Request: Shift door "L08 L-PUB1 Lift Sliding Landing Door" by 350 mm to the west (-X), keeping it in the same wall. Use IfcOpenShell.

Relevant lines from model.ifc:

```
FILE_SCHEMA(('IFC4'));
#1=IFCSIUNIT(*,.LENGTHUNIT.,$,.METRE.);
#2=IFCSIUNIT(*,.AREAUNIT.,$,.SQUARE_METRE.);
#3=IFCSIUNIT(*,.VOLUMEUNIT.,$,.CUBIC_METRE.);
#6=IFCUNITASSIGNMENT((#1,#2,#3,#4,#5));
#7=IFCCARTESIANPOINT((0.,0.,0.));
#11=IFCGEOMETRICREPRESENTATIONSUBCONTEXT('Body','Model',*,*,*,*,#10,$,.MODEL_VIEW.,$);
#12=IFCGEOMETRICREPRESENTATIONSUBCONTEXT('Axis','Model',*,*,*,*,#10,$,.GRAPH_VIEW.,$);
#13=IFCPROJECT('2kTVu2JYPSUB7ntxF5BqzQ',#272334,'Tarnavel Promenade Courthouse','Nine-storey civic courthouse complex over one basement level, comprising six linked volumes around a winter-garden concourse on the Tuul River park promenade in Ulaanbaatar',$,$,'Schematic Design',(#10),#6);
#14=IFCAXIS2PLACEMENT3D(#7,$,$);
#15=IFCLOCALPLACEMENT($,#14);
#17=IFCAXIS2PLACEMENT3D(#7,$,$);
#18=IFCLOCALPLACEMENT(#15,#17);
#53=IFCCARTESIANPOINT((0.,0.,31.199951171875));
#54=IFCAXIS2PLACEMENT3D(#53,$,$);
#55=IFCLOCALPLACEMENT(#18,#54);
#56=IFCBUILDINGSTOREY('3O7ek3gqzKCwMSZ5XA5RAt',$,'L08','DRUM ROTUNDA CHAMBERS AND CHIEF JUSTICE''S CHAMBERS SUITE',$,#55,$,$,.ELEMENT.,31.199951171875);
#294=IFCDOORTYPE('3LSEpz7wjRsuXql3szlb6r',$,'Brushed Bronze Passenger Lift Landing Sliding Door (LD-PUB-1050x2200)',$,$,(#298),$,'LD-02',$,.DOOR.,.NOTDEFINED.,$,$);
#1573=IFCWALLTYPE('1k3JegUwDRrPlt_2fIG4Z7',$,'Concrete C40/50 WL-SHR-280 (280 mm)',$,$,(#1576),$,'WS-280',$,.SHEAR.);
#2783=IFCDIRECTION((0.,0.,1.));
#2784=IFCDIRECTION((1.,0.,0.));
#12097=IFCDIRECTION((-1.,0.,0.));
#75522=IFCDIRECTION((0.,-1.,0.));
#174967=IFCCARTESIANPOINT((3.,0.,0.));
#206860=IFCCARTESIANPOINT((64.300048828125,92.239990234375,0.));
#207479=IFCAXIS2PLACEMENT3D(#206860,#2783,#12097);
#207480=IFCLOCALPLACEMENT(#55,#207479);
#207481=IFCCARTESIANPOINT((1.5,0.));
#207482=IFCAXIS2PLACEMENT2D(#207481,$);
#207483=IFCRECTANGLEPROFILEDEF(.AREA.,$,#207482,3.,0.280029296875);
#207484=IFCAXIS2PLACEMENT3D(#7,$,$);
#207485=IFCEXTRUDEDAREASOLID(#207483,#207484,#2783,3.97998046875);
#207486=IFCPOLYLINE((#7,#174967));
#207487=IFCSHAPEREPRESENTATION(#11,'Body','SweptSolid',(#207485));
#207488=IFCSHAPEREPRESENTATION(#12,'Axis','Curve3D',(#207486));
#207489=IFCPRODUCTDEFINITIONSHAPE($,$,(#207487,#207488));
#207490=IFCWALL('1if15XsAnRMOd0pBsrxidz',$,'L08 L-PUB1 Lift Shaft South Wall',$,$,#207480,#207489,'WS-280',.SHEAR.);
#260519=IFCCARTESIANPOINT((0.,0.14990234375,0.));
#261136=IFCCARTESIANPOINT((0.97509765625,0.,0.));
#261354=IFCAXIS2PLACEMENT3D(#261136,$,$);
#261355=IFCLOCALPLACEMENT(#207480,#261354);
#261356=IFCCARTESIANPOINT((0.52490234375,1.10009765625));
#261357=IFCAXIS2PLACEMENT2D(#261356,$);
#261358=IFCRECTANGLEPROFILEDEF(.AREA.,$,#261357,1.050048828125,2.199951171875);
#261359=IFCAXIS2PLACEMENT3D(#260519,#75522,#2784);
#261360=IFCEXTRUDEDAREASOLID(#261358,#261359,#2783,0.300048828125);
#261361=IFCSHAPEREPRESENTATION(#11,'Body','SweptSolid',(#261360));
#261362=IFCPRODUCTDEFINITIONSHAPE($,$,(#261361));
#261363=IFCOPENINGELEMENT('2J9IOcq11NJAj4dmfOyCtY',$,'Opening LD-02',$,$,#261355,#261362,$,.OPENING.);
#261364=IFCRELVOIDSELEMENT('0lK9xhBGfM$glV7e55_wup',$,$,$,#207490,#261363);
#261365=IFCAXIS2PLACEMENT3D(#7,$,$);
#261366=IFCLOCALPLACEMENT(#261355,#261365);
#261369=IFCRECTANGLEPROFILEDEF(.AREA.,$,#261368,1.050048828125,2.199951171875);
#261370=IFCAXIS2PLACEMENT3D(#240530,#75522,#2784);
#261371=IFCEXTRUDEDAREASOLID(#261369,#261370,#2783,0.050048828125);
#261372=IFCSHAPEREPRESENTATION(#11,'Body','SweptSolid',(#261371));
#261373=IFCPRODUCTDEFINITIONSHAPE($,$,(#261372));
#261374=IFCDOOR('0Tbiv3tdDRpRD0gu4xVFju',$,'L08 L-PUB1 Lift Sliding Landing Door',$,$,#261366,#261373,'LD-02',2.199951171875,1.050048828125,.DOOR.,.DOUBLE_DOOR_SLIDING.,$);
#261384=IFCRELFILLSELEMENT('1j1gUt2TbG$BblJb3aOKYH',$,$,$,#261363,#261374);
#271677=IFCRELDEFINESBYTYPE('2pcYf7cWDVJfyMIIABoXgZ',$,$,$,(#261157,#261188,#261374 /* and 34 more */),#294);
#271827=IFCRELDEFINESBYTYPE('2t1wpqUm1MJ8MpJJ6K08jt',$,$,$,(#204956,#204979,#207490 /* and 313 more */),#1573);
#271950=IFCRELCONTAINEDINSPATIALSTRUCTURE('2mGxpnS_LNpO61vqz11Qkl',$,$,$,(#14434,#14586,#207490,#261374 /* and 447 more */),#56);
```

```python
import ifcopenshell
import ifcopenshell.api.geometry
import ifcopenshell.util.placement
import ifcopenshell.util.unit

model = ifcopenshell.open("model.ifc")
unit_scale = ifcopenshell.util.unit.calculate_unit_scale(model)

door = model.by_guid("0Tbiv3tdDRpRD0gu4xVFju")
opening = door.FillsVoids[0].RelatingOpeningElement
wall = opening.VoidsElements[0].RelatingBuildingElement

wall_matrix = ifcopenshell.util.placement.get_local_placement(wall.ObjectPlacement)
shift = wall_matrix[:3, 0] * 0.35 / unit_scale
before = ifcopenshell.util.placement.get_local_placement(door.ObjectPlacement)[:3, 3].copy()

# The door is placed relative to its opening, so it follows when the opening moves.
matrix = ifcopenshell.util.placement.get_local_placement(opening.ObjectPlacement)
matrix[:3, 3] += shift
ifcopenshell.api.geometry.edit_object_placement(
    model, product=opening, matrix=matrix, is_si=False, should_transform_children=True
)

after = ifcopenshell.util.placement.get_local_placement(door.ObjectPlacement)[:3, 3]
print("door moved by", (after - before).round(3) + 0.0)

model.write("model-out.ifc")
```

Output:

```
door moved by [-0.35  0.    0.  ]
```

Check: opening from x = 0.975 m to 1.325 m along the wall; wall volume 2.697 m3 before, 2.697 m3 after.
